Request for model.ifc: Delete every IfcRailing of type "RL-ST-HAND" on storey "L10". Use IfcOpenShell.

First a look at what the model holds.

```python
import ifcopenshell
import ifcopenshell.util.element

model = ifcopenshell.open("model.ifc")
print(model.schema)
storey = next(s for s in model.by_type("IfcBuildingStorey") if s.Name == "L10")
railings = [e for e in ifcopenshell.util.element.get_decomposition(storey) if e.is_a("IfcRailing")]
seen = {}
for e in railings:
    element_type = ifcopenshell.util.element.get_type(e)
    name = element_type.Name if element_type not in (None, e) else None
    seen[name] = seen.get(name, 0) + 1
for name, count in sorted(seen.items(), key=str):
    print(count, "x", name)
```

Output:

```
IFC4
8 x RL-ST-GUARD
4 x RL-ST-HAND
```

```python
import ifcopenshell
import ifcopenshell.api.root
import ifcopenshell.util.element

model = ifcopenshell.open("model.ifc")

storey = next(s for s in model.by_type("IfcBuildingStorey") if s.Name == "L10")
railings = [e for e in ifcopenshell.util.element.get_decomposition(storey) if e.is_a("IfcRailing")]
targets = [e for e in railings if (t := ifcopenshell.util.element.get_type(e)) not in (None, e) and t.Name == "RL-ST-HAND"]

for e in targets:
    ifcopenshell.api.root.remove_product(model, product=e)
print(len(targets), "removed")

model.write("model-out.ifc")
```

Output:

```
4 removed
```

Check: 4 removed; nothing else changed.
